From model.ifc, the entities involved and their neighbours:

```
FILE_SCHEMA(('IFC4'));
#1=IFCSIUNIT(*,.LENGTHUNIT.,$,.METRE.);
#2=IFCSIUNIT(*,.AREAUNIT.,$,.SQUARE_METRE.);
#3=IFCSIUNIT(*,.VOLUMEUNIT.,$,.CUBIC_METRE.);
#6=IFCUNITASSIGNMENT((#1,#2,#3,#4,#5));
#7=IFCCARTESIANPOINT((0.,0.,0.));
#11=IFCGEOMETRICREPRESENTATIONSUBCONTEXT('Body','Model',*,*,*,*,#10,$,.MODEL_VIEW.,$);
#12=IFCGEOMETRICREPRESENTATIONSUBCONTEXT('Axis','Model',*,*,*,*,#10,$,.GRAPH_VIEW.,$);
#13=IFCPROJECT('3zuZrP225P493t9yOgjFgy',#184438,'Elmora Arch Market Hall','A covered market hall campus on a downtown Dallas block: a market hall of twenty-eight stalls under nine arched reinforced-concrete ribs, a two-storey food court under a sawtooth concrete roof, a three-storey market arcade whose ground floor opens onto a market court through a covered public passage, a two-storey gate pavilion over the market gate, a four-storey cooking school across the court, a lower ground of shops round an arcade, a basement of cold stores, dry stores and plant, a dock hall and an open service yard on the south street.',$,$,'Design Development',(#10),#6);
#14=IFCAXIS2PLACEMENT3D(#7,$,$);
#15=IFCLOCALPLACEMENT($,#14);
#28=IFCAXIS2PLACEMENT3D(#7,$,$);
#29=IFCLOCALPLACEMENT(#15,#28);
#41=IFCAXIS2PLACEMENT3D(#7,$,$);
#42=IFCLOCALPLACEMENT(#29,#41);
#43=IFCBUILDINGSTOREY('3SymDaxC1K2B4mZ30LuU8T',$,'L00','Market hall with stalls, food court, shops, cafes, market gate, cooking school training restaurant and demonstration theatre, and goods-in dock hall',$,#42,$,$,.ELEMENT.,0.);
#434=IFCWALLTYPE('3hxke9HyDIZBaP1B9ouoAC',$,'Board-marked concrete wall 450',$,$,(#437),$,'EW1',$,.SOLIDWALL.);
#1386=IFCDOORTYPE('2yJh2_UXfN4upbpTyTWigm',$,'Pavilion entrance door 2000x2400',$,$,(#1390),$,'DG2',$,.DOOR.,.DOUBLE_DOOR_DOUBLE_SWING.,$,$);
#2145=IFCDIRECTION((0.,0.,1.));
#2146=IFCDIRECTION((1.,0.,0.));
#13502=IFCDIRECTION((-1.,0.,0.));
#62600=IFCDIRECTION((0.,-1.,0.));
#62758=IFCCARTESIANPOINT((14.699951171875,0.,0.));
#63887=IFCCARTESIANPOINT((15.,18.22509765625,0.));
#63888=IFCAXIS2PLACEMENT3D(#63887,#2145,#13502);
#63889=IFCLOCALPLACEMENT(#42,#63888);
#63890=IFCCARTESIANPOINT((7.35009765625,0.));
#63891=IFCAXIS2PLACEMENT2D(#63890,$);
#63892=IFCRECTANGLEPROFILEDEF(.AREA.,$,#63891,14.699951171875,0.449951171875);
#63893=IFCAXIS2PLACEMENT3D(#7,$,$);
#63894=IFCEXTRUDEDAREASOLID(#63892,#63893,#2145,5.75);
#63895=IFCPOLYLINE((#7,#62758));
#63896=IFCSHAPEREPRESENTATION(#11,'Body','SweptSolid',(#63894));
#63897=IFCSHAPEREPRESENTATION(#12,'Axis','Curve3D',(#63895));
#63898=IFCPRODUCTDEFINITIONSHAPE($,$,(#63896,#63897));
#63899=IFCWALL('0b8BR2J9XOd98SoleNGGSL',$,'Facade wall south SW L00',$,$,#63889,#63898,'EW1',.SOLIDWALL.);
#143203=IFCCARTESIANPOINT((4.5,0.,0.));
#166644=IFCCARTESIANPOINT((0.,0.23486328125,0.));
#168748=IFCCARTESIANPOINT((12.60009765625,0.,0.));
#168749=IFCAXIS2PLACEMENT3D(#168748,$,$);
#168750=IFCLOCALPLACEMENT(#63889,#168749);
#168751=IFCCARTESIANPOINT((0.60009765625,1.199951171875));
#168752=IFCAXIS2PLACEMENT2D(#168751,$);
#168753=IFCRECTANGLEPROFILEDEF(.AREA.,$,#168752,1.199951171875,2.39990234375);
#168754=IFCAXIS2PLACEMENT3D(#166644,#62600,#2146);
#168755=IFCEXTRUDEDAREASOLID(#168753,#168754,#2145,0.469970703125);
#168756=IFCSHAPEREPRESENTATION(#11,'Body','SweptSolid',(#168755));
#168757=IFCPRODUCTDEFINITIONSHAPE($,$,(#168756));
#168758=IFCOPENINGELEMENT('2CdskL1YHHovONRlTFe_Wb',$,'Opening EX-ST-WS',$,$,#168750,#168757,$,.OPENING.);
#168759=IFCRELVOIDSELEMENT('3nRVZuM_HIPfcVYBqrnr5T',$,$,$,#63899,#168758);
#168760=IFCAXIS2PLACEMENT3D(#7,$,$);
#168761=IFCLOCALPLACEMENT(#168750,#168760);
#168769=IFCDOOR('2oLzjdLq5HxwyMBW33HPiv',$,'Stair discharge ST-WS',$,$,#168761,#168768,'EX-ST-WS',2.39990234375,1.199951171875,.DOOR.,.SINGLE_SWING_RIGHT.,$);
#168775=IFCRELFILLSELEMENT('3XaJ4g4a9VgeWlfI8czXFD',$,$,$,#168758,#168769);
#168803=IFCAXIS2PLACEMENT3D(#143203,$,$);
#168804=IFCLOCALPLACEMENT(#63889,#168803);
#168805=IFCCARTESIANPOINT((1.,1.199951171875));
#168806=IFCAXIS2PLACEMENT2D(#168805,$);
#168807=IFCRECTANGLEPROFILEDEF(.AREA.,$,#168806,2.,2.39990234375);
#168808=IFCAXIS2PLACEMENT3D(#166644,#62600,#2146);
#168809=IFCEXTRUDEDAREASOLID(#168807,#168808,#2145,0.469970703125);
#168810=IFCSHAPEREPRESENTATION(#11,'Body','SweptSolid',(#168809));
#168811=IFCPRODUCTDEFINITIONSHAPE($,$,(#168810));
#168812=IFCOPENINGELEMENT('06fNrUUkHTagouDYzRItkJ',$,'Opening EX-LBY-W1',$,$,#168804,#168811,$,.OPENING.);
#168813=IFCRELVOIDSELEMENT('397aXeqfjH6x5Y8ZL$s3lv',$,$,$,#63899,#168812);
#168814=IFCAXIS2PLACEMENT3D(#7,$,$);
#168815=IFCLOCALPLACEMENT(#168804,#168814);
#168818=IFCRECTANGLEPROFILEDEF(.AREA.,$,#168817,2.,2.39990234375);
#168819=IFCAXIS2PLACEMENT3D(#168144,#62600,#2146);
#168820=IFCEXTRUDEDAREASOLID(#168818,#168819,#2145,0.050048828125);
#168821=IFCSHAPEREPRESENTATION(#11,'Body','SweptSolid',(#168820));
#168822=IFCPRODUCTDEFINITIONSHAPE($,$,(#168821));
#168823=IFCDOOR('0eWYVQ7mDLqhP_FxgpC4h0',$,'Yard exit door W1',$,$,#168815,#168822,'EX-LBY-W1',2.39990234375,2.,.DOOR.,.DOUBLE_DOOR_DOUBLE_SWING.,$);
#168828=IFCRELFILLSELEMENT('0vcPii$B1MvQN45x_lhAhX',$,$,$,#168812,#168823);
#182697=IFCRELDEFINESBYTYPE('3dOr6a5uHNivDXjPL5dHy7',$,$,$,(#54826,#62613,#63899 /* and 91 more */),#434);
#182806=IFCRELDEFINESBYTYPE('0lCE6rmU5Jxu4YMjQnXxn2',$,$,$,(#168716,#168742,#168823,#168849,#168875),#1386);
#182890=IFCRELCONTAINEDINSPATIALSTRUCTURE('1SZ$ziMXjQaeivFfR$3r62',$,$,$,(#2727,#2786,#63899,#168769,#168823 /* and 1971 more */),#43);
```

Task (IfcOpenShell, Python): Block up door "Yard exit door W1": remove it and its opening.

```python
import ifcopenshell
import ifcopenshell.api.feature
import ifcopenshell.api.root
import ifcopenshell.geom
import ifcopenshell.util.shape

model = ifcopenshell.open("model.ifc")
settings = ifcopenshell.geom.settings()


def volume(element):
    """Net volume in cubic metres, openings subtracted."""
    shape = ifcopenshell.geom.create_shape(settings, element)
    return ifcopenshell.util.shape.get_volume(shape.geometry)


door = model.by_guid("0eWYVQ7mDLqhP_FxgpC4h0")
opening = door.FillsVoids[0].RelatingOpeningElement
wall = opening.VoidsElements[0].RelatingBuildingElement
before = volume(wall)

ifcopenshell.api.root.remove_product(model, product=door)
ifcopenshell.api.feature.remove_feature(model, feature=opening)

after = volume(wall)

print(f"wall volume {before:.3f} -> {after:.3f} m3")

model.write("model_v2.ifc")
```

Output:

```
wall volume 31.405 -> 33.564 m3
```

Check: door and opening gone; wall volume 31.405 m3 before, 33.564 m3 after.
